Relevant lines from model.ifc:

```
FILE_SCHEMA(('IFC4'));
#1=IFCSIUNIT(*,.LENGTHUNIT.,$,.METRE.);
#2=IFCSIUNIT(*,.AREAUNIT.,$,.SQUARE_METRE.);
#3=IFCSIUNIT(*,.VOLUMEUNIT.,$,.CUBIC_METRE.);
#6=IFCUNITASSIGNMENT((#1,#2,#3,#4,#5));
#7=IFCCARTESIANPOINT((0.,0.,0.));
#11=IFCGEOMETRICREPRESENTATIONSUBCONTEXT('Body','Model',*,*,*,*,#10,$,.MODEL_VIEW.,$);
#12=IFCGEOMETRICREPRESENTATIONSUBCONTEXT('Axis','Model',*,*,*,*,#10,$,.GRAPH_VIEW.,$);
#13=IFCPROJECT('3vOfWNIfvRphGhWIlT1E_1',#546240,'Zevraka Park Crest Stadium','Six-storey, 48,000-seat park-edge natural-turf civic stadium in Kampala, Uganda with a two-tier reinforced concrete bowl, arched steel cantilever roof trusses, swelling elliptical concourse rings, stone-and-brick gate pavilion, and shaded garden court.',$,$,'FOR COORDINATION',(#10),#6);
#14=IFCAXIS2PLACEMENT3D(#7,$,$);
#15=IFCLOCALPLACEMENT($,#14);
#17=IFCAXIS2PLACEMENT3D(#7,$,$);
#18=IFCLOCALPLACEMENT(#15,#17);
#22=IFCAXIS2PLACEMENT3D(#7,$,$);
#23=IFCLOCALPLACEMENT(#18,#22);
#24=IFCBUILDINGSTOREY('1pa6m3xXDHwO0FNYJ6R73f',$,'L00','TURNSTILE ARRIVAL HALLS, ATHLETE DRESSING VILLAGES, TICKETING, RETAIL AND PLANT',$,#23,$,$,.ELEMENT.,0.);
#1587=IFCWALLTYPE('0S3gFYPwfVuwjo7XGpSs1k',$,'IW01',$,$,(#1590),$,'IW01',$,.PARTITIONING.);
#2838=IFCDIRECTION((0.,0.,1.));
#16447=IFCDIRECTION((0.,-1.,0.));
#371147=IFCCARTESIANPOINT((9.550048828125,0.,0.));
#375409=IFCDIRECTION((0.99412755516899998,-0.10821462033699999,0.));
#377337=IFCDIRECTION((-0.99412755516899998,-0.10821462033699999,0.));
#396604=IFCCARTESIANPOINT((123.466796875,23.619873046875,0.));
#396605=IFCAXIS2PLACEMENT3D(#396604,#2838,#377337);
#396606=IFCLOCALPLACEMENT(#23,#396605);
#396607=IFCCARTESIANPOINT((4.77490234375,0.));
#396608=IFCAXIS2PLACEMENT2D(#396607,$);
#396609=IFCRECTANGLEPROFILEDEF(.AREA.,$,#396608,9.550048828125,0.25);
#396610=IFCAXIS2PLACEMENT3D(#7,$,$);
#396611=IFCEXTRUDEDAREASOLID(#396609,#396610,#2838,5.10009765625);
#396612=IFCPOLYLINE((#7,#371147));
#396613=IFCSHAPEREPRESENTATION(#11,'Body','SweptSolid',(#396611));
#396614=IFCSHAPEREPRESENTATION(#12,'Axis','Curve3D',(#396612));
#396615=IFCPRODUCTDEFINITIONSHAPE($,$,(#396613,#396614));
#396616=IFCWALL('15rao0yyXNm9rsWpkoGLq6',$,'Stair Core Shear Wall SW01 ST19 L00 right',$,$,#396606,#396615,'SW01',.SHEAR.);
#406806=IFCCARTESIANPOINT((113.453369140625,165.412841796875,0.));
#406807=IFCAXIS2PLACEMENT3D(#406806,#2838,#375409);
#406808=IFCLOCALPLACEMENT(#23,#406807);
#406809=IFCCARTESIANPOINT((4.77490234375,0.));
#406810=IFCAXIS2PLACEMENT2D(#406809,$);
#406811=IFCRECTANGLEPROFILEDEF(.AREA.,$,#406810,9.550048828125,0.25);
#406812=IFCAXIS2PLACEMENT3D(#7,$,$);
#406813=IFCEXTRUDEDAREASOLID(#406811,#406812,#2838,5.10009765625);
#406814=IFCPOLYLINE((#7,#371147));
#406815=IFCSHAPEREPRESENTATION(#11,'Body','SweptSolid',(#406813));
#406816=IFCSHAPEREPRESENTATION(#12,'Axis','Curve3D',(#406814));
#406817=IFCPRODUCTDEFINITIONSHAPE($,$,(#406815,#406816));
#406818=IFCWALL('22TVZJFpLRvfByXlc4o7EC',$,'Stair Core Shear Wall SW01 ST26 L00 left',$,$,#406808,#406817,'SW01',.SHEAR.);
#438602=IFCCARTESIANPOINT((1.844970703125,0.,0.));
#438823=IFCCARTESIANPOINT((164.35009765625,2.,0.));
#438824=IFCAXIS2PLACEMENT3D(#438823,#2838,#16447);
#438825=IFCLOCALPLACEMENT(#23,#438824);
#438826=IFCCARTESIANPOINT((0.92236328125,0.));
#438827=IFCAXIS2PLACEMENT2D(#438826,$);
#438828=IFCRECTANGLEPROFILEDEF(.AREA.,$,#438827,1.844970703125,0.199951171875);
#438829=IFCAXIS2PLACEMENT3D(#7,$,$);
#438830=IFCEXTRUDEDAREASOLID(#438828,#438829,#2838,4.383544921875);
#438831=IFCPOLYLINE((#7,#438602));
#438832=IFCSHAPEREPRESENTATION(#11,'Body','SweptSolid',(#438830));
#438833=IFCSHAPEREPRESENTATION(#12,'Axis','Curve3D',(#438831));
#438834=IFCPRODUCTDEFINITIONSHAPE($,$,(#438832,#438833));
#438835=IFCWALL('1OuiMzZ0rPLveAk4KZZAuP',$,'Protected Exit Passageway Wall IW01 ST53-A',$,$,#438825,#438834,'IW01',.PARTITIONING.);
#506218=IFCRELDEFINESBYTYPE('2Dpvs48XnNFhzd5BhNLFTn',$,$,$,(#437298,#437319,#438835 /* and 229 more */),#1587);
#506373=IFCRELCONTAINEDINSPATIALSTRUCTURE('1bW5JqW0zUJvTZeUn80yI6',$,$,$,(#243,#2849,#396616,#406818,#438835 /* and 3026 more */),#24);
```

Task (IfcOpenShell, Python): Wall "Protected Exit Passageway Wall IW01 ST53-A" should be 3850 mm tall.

```python
import ifcopenshell
import ifcopenshell.geom
import ifcopenshell.util.representation
import ifcopenshell.util.shape
import ifcopenshell.util.unit

model = ifcopenshell.open("model.ifc")
unit_scale = ifcopenshell.util.unit.calculate_unit_scale(model)
settings = ifcopenshell.geom.settings()


def volume(element):
    """Net volume in cubic metres, openings subtracted."""
    shape = ifcopenshell.geom.create_shape(settings, element)
    return ifcopenshell.util.shape.get_volume(shape.geometry)


wall = model.by_id(438835)
before = volume(wall)

body = ifcopenshell.util.representation.get_representation(wall, "Model", "Body")
solid = body.Items[0]
old_height = solid.Depth
solid.Depth = 3.85 / unit_scale
after = volume(wall)

print(f"height {old_height:g} -> {solid.Depth:g}, volume {before:.3f} -> {after:.3f} m3")

model.write("model-out.ifc")
```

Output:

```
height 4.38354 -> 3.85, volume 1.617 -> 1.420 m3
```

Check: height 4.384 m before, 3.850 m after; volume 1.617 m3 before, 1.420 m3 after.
